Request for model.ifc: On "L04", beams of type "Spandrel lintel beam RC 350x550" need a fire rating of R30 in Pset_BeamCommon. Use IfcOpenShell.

First a look at what the model holds.

```python
import ifcopenshell
import ifcopenshell.util.element

model = ifcopenshell.open("model.ifc")
print(model.schema)
storey = next(s for s in model.by_type("IfcBuildingStorey") if s.Name == "L04")
beams = [e for e in ifcopenshell.util.element.get_decomposition(storey) if e.is_a("IfcBeam")]
seen = {}
for e in beams:
    element_type = ifcopenshell.util.element.get_type(e)
    key = (element_type.Name if element_type != e and element_type else None, ifcopenshell.util.element.get_pset(e, "Pset_BeamCommon", "FireRating"))
    seen[key] = seen.get(key, 0) + 1
for (name, value), count in sorted(seen.items(), key=str):
    print(count, "x", name, "|", value)
```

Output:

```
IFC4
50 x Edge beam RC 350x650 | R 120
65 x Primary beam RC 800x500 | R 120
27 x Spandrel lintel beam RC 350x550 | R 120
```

```python
import ifcopenshell
import ifcopenshell.api.pset
import ifcopenshell.util.element

model = ifcopenshell.open("model.ifc")

storey = next(s for s in model.by_type("IfcBuildingStorey") if s.Name == "L04")
beams = [e for e in ifcopenshell.util.element.get_decomposition(storey) if e.is_a("IfcBeam")]

count = 0
for e in beams:
    element_type = ifcopenshell.util.element.get_type(e)
    if element_type in (None, e) or element_type.Name != "Spandrel lintel beam RC 350x550":
        continue
    # add_pset returns the element's existing set when there is one.
    pset = ifcopenshell.api.pset.add_pset(model, product=e, name="Pset_BeamCommon")
    ifcopenshell.api.pset.edit_pset(model, pset=pset, properties={"FireRating": "R30"})
    count += 1

print(count, "beams updated")

model.write("model-out.ifc")
```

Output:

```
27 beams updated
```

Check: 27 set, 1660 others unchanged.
